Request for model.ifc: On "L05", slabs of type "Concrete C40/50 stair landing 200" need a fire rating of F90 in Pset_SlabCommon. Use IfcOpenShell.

First a look at what the model holds.

```python
import ifcopenshell
import ifcopenshell.util.element

model = ifcopenshell.open("model.ifc")
print(model.schema)
storey = next(s for s in model.by_type("IfcBuildingStorey") if s.Name == "L05")
slabs = [e for e in ifcopenshell.util.element.get_decomposition(storey) if e.is_a("IfcSlab")]
seen = {}
for e in slabs:
    element_type = ifcopenshell.util.element.get_type(e)
    key = (element_type.Name if element_type != e and element_type else None, ifcopenshell.util.element.get_pset(e, "Pset_SlabCommon", "FireRating"))
    seen[key] = seen.get(key, 0) + 1
for (name, value), count in sorted(seen.items(), key=str):
    print(count, "x", name, "|", value)
```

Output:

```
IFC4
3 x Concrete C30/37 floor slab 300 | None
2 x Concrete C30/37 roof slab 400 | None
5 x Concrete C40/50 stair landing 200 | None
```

```python
import ifcopenshell
import ifcopenshell.api.pset
import ifcopenshell.util.element

model = ifcopenshell.open("model.ifc")

storey = next(s for s in model.by_type("IfcBuildingStorey") if s.Name == "L05")
slabs = [e for e in ifcopenshell.util.element.get_decomposition(storey) if e.is_a("IfcSlab")]

count = 0
for e in slabs:
    element_type = ifcopenshell.util.element.get_type(e)
    if element_type in (None, e) or element_type.Name != "Concrete C40/50 stair landing 200":
        continue
    # add_pset returns the element's existing set when there is one.
    pset = ifcopenshell.api.pset.add_pset(model, product=e, name="Pset_SlabCommon")
    ifcopenshell.api.pset.edit_pset(model, pset=pset, properties={"FireRating": "F90"})
    count += 1

print(count, "slabs updated")

model.write("model_rev.ifc")
```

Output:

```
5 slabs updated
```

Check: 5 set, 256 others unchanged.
